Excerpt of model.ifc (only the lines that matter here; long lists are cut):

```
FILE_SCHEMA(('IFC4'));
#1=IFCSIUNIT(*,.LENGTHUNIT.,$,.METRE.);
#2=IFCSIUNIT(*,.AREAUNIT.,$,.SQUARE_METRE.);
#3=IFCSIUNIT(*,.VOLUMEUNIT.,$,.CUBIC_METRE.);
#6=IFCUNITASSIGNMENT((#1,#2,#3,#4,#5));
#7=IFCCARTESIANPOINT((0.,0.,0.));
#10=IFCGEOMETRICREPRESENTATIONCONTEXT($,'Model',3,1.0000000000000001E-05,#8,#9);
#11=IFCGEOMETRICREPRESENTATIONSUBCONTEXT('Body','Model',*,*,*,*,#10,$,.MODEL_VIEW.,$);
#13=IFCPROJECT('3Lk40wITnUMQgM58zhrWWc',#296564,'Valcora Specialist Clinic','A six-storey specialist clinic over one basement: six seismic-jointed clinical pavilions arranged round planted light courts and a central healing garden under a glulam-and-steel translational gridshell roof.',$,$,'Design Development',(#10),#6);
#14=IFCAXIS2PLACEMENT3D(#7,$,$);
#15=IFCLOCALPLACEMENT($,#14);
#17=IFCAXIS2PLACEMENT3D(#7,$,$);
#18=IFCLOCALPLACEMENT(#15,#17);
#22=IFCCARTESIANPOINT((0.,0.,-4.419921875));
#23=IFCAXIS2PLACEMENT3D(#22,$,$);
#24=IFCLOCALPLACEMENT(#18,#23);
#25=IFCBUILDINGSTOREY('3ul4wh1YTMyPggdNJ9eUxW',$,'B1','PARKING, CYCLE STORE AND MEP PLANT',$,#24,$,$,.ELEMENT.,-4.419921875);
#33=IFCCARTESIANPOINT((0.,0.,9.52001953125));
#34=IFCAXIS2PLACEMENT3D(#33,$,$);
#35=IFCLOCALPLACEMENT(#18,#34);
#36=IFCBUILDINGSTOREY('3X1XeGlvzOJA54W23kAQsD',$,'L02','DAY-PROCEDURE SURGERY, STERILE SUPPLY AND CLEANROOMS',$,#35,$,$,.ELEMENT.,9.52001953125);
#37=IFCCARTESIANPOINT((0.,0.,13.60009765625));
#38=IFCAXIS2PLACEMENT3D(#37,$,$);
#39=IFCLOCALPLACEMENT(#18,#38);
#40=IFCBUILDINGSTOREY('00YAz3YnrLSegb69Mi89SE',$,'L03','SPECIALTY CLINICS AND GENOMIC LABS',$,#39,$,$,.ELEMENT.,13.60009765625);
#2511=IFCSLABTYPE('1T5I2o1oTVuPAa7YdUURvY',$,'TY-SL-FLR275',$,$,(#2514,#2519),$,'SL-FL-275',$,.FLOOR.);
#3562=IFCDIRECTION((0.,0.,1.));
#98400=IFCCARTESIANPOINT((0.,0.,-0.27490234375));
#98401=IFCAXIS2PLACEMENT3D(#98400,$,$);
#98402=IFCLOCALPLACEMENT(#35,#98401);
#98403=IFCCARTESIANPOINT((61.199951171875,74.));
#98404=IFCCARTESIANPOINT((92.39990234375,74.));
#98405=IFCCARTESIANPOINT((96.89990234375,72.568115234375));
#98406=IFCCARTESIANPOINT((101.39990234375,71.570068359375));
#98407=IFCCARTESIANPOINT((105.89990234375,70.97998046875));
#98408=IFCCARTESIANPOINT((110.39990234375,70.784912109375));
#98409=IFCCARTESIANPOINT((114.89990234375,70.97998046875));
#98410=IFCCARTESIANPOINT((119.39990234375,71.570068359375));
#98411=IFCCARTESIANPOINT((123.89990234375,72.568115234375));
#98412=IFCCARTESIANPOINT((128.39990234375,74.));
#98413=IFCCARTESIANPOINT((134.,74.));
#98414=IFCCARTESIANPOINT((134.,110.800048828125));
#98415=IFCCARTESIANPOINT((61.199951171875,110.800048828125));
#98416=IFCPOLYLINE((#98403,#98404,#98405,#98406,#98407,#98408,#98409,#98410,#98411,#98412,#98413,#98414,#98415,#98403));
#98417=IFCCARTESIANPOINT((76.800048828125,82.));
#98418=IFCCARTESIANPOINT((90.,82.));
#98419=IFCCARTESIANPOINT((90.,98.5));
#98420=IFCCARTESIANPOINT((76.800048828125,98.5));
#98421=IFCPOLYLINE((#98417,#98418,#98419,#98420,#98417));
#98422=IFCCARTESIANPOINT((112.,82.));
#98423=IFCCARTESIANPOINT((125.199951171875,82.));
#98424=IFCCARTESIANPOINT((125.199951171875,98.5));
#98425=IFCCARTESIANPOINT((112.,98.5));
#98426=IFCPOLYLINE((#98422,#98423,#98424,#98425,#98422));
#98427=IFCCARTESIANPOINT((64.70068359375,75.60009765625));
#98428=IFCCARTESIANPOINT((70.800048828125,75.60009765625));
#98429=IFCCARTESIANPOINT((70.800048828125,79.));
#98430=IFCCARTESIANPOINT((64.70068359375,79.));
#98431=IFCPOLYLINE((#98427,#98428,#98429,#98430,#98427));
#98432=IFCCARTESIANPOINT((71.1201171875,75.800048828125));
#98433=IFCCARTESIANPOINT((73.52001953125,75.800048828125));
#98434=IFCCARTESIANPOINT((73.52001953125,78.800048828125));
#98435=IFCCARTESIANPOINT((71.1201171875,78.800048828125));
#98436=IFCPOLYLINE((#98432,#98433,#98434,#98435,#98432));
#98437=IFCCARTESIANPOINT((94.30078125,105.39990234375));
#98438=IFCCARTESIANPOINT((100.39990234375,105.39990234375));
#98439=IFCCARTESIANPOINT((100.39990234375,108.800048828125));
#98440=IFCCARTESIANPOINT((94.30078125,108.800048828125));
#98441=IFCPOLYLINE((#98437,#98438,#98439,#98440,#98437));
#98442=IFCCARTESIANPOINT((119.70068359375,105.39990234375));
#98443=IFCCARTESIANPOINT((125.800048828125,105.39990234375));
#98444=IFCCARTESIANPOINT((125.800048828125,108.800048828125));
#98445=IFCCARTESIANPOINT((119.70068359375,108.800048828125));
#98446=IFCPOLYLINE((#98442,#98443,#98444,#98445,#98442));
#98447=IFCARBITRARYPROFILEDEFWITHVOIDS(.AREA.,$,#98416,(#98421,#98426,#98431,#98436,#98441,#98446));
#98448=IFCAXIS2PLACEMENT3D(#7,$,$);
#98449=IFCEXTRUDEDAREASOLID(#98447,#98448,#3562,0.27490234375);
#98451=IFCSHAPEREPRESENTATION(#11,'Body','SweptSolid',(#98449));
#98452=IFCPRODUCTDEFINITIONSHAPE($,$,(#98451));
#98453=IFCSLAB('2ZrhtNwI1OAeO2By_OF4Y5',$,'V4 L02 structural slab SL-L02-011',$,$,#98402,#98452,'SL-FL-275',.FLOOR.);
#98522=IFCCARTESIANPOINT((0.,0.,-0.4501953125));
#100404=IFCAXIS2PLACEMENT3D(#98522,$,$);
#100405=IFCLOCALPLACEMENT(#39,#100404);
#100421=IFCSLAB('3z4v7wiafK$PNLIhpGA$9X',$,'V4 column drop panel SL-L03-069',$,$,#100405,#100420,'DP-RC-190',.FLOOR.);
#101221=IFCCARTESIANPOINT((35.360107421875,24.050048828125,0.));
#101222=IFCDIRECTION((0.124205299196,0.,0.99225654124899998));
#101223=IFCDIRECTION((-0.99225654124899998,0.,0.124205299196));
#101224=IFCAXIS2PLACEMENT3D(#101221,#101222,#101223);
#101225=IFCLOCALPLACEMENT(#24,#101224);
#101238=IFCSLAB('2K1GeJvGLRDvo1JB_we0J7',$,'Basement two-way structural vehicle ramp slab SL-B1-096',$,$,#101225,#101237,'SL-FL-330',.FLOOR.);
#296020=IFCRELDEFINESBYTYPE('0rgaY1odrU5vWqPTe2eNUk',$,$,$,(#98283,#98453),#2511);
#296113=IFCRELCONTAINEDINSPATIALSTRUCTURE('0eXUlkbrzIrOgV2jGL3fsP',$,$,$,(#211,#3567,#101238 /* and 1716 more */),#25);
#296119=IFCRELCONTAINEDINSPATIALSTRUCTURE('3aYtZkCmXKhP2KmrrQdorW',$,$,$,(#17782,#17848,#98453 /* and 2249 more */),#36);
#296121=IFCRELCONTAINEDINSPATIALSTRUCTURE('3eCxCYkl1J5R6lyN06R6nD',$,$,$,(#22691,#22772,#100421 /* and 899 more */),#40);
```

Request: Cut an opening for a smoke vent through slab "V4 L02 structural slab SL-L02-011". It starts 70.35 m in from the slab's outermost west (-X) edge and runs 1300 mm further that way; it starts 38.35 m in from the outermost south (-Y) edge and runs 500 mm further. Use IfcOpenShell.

```python
import numpy as np
import ifcopenshell
import ifcopenshell.api.feature
import ifcopenshell.api.geometry
import ifcopenshell.api.root
import ifcopenshell.geom
import ifcopenshell.util.placement
import ifcopenshell.util.representation
import ifcopenshell.util.shape
import ifcopenshell.util.unit

model = ifcopenshell.open("model.ifc")
unit_scale = ifcopenshell.util.unit.calculate_unit_scale(model)
settings = ifcopenshell.geom.settings()


def volume(element):
    """Net volume in cubic metres, openings subtracted."""
    shape = ifcopenshell.geom.create_shape(settings, element)
    return ifcopenshell.util.shape.get_volume(shape.geometry)


slab = model.by_guid("2ZrhtNwI1OAeO2By_OF4Y5")
before = volume(slab)

# Extent in the slab's own axes, in metres. The edges named are its -X and -Y sides.
slab_shape = ifcopenshell.geom.create_shape(settings, slab)
vertices = ifcopenshell.util.shape.get_vertices(slab_shape.geometry)
x_min, y_min, bottom = vertices.min(axis=0)
top = vertices[:, 2].max()

opening = ifcopenshell.api.root.create_entity(model, ifc_class="IfcOpeningElement", name="Smoke vent opening", predefined_type="OPENING")
context = ifcopenshell.util.representation.get_context(model, "Model", "Body", "MODEL_VIEW")
width, depth = 1.3, 0.5
outline = [(0.0, 0.0), (width, 0.0), (width, depth), (0.0, depth), (0.0, 0.0)]
# Overshoot both faces by 50 mm so the cut is clean.
shape = ifcopenshell.api.geometry.add_slab_representation(
    model, context=context, depth=top - bottom + 0.1, polyline=outline
)
ifcopenshell.api.geometry.assign_representation(model, product=opening, representation=shape)

matrix = ifcopenshell.util.placement.get_local_placement(slab.ObjectPlacement)
matrix[:, 3] = matrix @ np.append(np.array([x_min + 70.35, y_min + 38.35, bottom - 0.05]) / unit_scale, 1.0)
ifcopenshell.api.geometry.edit_object_placement(model, product=opening, matrix=matrix, is_si=False)
ifcopenshell.api.feature.add_feature(model, feature=opening, element=slab)

after = volume(slab)

print(f"slab volume {before:.3f} -> {after:.3f} m3")

model.write("model_edited.ifc")
```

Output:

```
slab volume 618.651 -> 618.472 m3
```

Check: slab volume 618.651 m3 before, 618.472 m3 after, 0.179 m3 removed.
